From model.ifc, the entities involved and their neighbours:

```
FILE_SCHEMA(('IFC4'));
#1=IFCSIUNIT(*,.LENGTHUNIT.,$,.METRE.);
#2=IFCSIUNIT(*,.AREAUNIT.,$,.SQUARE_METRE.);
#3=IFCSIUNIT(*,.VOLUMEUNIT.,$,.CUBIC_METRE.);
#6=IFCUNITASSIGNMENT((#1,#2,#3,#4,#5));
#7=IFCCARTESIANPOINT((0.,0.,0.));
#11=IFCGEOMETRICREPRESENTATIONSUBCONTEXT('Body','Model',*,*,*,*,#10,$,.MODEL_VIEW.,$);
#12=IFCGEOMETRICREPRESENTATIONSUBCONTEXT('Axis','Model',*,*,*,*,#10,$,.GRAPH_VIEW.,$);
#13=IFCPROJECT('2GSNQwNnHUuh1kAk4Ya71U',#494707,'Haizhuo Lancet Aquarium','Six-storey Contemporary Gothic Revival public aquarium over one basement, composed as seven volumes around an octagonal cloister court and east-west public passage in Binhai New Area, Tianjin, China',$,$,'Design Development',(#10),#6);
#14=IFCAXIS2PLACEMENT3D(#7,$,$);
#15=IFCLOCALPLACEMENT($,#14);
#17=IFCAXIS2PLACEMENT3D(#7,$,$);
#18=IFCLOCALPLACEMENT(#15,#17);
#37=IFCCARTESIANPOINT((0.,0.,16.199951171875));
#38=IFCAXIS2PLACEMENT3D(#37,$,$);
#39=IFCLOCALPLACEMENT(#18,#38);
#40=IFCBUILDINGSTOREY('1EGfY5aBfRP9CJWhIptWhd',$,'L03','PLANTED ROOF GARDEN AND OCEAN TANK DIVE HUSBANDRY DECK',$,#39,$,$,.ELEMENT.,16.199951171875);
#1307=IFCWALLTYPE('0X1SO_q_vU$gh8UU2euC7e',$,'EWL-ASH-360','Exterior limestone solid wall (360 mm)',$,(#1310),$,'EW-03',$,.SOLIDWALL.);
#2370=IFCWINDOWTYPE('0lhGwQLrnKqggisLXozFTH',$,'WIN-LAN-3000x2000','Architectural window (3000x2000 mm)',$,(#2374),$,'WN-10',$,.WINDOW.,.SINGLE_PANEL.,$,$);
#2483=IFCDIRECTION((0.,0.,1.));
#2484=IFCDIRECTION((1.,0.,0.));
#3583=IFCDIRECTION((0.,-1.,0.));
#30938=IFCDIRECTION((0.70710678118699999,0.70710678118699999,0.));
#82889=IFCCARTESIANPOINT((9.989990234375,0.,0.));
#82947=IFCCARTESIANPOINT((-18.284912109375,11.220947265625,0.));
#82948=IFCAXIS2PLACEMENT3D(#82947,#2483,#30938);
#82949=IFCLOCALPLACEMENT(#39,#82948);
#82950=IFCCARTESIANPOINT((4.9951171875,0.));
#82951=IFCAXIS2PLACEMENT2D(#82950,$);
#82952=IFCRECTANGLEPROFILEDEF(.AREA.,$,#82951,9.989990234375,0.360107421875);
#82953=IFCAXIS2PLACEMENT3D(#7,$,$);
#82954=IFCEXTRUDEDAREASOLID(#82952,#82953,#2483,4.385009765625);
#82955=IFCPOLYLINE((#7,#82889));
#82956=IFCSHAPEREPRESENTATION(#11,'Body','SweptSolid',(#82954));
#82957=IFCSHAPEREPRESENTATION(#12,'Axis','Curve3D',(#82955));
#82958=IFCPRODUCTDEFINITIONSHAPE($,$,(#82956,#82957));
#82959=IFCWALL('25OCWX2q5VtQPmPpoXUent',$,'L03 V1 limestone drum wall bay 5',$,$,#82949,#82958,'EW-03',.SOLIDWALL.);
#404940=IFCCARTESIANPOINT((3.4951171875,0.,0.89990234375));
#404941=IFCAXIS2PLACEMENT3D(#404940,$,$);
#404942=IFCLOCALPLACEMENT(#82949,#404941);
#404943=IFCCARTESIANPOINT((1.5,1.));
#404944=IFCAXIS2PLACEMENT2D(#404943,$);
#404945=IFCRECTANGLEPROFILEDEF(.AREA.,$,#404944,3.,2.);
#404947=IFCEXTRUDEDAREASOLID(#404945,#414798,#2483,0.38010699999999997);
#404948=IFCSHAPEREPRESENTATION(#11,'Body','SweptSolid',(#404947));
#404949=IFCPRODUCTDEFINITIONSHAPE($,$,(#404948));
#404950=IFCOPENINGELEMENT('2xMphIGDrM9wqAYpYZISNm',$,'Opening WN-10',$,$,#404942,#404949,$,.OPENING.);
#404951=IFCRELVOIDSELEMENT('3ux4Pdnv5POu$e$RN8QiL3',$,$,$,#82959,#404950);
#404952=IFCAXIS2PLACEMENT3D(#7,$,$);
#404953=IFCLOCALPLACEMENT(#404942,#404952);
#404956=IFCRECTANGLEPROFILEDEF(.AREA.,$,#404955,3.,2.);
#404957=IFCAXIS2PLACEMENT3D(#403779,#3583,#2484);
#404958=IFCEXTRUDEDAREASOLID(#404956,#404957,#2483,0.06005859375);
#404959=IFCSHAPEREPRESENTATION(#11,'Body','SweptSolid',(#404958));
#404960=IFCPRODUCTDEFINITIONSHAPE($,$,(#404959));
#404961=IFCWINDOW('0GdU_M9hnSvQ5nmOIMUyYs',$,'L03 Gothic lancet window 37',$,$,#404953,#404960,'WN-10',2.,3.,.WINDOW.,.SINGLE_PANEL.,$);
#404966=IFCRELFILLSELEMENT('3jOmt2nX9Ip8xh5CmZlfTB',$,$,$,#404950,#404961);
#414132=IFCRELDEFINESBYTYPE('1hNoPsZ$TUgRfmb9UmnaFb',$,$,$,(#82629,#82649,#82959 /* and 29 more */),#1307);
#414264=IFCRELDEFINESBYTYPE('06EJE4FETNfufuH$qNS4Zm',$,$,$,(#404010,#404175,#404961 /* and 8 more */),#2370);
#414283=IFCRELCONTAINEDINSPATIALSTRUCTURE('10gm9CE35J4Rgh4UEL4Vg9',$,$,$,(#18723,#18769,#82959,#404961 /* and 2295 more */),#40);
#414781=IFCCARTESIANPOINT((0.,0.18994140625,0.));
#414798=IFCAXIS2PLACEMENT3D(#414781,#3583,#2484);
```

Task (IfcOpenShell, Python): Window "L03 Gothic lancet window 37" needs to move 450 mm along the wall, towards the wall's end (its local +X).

```python
import ifcopenshell
import ifcopenshell.api.geometry
import ifcopenshell.util.placement
import ifcopenshell.util.unit

model = ifcopenshell.open("model.ifc")
unit_scale = ifcopenshell.util.unit.calculate_unit_scale(model)

window = model.by_guid("0GdU_M9hnSvQ5nmOIMUyYs")
opening = window.FillsVoids[0].RelatingOpeningElement
wall = opening.VoidsElements[0].RelatingBuildingElement

wall_matrix = ifcopenshell.util.placement.get_local_placement(wall.ObjectPlacement)
shift = wall_matrix[:3, 0] * 0.45 / unit_scale
before = ifcopenshell.util.placement.get_local_placement(window.ObjectPlacement)[:3, 3].copy()

# The window is placed relative to its opening, so it follows when the opening moves.
matrix = ifcopenshell.util.placement.get_local_placement(opening.ObjectPlacement)
matrix[:3, 3] += shift
ifcopenshell.api.geometry.edit_object_placement(
    model, product=opening, matrix=matrix, is_si=False, should_transform_children=True
)

after = ifcopenshell.util.placement.get_local_placement(window.ObjectPlacement)[:3, 3]
print("window moved by", (after - before).round(3) + 0.0)

model.write("model-out.ifc")
```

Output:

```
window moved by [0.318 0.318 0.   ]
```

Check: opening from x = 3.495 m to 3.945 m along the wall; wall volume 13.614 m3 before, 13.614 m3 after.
